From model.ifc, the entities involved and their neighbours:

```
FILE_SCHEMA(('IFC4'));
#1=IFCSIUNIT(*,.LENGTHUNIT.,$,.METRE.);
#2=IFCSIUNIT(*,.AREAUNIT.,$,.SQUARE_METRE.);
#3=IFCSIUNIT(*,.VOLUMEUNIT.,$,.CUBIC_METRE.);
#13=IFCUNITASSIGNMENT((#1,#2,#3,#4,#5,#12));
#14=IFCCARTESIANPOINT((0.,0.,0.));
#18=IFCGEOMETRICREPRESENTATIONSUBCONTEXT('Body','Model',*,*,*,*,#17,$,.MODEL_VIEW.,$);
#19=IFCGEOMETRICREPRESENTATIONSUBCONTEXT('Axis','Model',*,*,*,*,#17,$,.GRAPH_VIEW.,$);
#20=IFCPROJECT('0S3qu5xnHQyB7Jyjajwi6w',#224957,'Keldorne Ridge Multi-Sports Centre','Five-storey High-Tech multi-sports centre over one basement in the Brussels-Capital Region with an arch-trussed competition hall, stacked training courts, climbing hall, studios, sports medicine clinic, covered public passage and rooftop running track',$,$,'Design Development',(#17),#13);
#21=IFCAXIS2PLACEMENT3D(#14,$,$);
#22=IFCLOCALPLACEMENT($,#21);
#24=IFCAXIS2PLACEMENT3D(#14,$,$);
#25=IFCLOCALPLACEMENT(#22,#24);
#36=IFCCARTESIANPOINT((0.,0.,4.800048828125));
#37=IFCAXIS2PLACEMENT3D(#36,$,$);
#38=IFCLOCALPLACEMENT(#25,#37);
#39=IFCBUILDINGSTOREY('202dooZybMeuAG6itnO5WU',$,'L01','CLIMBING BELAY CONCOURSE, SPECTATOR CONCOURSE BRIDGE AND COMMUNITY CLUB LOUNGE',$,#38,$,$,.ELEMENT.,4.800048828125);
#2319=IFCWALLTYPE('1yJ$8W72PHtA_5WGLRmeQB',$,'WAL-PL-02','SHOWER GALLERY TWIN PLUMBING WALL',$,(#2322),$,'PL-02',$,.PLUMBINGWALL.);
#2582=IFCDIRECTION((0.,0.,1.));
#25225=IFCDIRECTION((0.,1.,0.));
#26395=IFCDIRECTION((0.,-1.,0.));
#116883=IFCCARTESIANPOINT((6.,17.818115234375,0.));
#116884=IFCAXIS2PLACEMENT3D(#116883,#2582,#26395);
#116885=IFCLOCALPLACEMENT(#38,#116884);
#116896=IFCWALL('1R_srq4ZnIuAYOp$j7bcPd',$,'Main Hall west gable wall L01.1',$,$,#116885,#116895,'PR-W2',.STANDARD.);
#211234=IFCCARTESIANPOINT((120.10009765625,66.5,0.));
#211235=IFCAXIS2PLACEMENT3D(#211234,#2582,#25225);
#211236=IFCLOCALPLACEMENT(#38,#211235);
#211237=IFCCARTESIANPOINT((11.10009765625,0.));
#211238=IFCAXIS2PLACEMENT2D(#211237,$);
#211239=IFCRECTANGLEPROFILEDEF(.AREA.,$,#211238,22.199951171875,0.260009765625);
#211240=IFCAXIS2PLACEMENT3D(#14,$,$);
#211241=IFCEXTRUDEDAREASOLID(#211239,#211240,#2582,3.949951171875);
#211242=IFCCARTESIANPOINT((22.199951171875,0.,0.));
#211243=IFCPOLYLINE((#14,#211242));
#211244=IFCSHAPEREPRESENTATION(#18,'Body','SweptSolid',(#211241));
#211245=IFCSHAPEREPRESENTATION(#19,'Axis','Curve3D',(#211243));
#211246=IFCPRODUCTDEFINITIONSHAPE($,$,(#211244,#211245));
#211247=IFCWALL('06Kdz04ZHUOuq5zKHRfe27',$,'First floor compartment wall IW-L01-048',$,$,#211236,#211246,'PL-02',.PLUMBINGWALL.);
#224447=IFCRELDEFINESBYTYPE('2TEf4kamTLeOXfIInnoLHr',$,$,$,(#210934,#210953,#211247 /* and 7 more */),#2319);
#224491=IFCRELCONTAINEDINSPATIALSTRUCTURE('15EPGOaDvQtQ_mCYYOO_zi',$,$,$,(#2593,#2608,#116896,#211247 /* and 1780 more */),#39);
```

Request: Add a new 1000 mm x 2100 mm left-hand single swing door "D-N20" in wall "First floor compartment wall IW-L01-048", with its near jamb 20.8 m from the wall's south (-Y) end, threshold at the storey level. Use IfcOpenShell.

```python
import numpy as np
import ifcopenshell
import ifcopenshell.api.feature
import ifcopenshell.api.geometry
import ifcopenshell.api.root
import ifcopenshell.api.spatial
import ifcopenshell.geom
import ifcopenshell.util.element
import ifcopenshell.util.placement
import ifcopenshell.util.representation
import ifcopenshell.util.shape
import ifcopenshell.util.unit

model = ifcopenshell.open("model.ifc")
unit_scale = ifcopenshell.util.unit.calculate_unit_scale(model)
settings = ifcopenshell.geom.settings()


def volume(element):
    """Net volume in cubic metres, openings subtracted."""
    shape = ifcopenshell.geom.create_shape(settings, element)
    return ifcopenshell.util.shape.get_volume(shape.geometry)


wall = model.by_id(211247)
storey = ifcopenshell.util.element.get_container(wall, ifc_class="IfcBuildingStorey")
context = ifcopenshell.util.representation.get_context(model, "Model", "Body", "MODEL_VIEW")
before = volume(wall)

width, height, from_end, sill = 1, 2.1, 20.8, 0.0  # metres

# The wall runs along its own X axis, and the end named is its -X end.
wall_shape = ifcopenshell.geom.create_shape(settings, wall)
x, y, z = ifcopenshell.util.shape.get_vertices(wall_shape.geometry).T
start = x.min() + from_end
face, thickness = float(y.min()), float(y.max() - y.min())
wall_matrix = ifcopenshell.util.placement.get_local_placement(wall.ObjectPlacement)
level = ifcopenshell.util.placement.get_local_placement(storey.ObjectPlacement)[2, 3]


def in_wall(x, y):
    """Placement at x, y metres in the wall's axes, at sill height."""
    matrix = wall_matrix.copy()
    matrix[:, 3] = wall_matrix @ np.array([x / unit_scale, y / unit_scale, 0.0, 1.0])
    matrix[2, 3] = level + sill / unit_scale
    return matrix


# Opening: a box that overshoots both wall faces by 50 mm.
opening = ifcopenshell.api.root.create_entity(model, ifc_class="IfcOpeningElement", predefined_type="OPENING")
box = ifcopenshell.api.geometry.add_wall_representation(
    model, context=context, length=width, height=height, thickness=thickness + 0.1
)
ifcopenshell.api.geometry.assign_representation(model, product=opening, representation=box)
ifcopenshell.api.geometry.edit_object_placement(model, product=opening, matrix=in_wall(start, face - 0.05), is_si=False)
ifcopenshell.api.feature.add_feature(model, feature=opening, element=wall)

door = ifcopenshell.api.root.create_entity(model, ifc_class="IfcDoor", name="D-N20", predefined_type="DOOR")
door.OverallWidth, door.OverallHeight = width / unit_scale, height / unit_scale
door.OperationType = "SINGLE_SWING_LEFT"
body = ifcopenshell.api.geometry.add_door_representation(
    model,
    context=context,
    overall_width=door.OverallWidth,
    overall_height=door.OverallHeight,
    operation_type="SINGLE_SWING_LEFT",
    lining_properties={"LiningDepth": thickness / unit_scale, "ThresholdDepth": thickness / unit_scale},
)
ifcopenshell.api.geometry.assign_representation(model, product=door, representation=body)
ifcopenshell.api.spatial.assign_container(model, products=[door], relating_structure=storey)
ifcopenshell.api.feature.add_filling(model, opening=opening, element=door)

# The lining spans the wall, so the door starts at the wall face.
ifcopenshell.api.geometry.edit_object_placement(model, product=door, matrix=in_wall(start, face), is_si=False)

after = volume(wall)

print(f"wall volume {before:.3f} -> {after:.3f} m3")

model.write("model_rev.ifc")
```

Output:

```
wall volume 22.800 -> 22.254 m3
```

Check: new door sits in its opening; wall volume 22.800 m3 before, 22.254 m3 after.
